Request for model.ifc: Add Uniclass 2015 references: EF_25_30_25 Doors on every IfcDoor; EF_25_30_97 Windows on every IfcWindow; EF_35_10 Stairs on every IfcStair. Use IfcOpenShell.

First a look at what the model holds.

```python
import ifcopenshell

model = ifcopenshell.open("model.ifc")
print(model.schema)
print("classifications:", [c.Name for c in model.by_type("IfcClassification")])
for ifc_class in ("IfcDoor", "IfcRoof", "IfcStair", "IfcWall", "IfcWindow"):
    print(ifc_class, len(model.by_type(ifc_class)))
```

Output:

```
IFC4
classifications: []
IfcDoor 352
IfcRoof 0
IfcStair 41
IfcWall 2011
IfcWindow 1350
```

```python
import ifcopenshell
import ifcopenshell.api.classification

model = ifcopenshell.open("model.ifc")

system = ifcopenshell.api.classification.add_classification(model, classification="Uniclass 2015")

codes = {
    "IfcDoor": ("EF_25_30_25", "Doors"),
    "IfcWindow": ("EF_25_30_97", "Windows"),
    "IfcStair": ("EF_35_10", "Stairs"),
}
for ifc_class, (code, name) in codes.items():
    products = model.by_type(ifc_class)
    ifcopenshell.api.classification.add_reference(
        model, products=products, classification=system, identification=code, name=name
    )
    print(code, len(products))

model.write("model-out.ifc")
```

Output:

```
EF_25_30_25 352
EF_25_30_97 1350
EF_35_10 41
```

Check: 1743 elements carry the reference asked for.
